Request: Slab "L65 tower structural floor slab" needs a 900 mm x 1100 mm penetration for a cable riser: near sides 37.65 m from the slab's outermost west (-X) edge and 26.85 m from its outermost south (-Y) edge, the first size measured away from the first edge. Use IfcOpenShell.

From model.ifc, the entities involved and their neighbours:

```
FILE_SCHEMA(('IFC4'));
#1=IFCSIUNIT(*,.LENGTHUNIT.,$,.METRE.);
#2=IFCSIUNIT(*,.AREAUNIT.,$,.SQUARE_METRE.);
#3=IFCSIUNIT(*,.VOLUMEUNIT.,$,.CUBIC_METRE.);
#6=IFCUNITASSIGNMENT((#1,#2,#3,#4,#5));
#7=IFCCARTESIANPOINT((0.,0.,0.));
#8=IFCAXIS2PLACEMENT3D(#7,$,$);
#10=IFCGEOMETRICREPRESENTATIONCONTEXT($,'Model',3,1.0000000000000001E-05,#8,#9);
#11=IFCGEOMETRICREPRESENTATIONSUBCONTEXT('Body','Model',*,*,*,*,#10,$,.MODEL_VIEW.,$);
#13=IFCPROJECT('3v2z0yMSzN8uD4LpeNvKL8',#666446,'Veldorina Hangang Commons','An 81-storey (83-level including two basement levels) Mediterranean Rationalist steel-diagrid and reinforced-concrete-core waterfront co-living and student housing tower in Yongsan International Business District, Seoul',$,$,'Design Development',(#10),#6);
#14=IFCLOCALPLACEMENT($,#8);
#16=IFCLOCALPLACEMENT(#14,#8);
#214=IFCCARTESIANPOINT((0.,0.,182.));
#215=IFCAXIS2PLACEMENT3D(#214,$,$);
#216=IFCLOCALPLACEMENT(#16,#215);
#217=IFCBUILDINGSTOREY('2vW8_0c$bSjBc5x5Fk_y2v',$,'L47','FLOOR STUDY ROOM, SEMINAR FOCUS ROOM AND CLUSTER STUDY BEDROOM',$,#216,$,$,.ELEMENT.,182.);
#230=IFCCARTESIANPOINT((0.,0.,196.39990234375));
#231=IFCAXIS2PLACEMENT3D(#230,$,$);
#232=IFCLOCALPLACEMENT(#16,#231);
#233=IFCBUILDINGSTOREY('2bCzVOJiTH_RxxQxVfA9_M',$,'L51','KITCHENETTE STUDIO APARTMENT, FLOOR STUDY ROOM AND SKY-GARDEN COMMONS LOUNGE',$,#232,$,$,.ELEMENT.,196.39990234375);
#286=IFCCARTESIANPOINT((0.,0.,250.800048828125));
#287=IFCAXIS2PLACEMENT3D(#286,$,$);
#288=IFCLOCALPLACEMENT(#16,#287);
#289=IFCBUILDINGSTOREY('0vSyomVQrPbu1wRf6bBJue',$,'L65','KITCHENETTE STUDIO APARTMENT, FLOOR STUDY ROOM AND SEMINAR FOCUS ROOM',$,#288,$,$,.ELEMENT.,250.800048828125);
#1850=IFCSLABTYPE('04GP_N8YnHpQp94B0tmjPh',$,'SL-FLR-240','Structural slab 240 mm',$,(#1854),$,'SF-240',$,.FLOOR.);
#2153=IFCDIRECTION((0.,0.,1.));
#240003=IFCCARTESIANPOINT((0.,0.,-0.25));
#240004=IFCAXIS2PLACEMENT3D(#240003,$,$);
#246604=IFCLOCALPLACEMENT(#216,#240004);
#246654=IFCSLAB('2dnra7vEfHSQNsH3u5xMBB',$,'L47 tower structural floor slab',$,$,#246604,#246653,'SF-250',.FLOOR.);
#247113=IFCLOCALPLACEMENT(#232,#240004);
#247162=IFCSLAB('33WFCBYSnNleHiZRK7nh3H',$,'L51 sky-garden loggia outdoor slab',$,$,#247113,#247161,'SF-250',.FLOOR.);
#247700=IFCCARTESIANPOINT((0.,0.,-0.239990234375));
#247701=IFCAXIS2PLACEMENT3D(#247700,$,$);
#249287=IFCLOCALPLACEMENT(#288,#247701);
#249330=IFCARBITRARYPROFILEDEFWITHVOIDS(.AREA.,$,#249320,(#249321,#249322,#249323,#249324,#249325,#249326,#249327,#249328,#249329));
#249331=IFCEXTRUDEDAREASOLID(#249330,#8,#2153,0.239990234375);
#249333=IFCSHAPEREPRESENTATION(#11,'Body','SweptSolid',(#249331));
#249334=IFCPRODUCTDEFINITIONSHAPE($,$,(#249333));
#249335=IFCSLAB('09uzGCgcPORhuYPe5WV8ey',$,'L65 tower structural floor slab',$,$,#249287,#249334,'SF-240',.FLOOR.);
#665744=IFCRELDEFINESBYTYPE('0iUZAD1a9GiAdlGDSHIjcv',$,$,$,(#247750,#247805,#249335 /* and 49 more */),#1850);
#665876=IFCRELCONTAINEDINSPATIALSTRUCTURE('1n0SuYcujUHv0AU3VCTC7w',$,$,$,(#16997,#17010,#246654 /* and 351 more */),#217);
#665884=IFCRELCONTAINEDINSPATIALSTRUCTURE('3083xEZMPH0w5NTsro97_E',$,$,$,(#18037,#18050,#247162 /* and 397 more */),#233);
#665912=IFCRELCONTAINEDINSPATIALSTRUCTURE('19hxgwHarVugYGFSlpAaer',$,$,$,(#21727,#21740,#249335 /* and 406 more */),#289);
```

```python
import numpy as np
import ifcopenshell
import ifcopenshell.api.feature
import ifcopenshell.api.geometry
import ifcopenshell.api.root
import ifcopenshell.geom
import ifcopenshell.util.placement
import ifcopenshell.util.representation
import ifcopenshell.util.shape
import ifcopenshell.util.unit

model = ifcopenshell.open("model.ifc")
unit_scale = ifcopenshell.util.unit.calculate_unit_scale(model)
settings = ifcopenshell.geom.settings()


def volume(element):
    """Net volume in cubic metres, openings subtracted."""
    shape = ifcopenshell.geom.create_shape(settings, element)
    return ifcopenshell.util.shape.get_volume(shape.geometry)


slab = model.by_id(249335)
before = volume(slab)

# Extent in the slab's own axes, in metres. The edges named are its -X and -Y sides.
slab_shape = ifcopenshell.geom.create_shape(settings, slab)
vertices = ifcopenshell.util.shape.get_vertices(slab_shape.geometry)
x_min, y_min, bottom = vertices.min(axis=0)
top = vertices[:, 2].max()

opening = ifcopenshell.api.root.create_entity(model, ifc_class="IfcOpeningElement", name="Cable riser opening", predefined_type="OPENING")
context = ifcopenshell.util.representation.get_context(model, "Model", "Body", "MODEL_VIEW")
width, depth = 0.9, 1.1
outline = [(0.0, 0.0), (width, 0.0), (width, depth), (0.0, depth), (0.0, 0.0)]
# Overshoot both faces by 50 mm so the cut is clean.
shape = ifcopenshell.api.geometry.add_slab_representation(
    model, context=context, depth=top - bottom + 0.1, polyline=outline
)
ifcopenshell.api.geometry.assign_representation(model, product=opening, representation=shape)

matrix = ifcopenshell.util.placement.get_local_placement(slab.ObjectPlacement)
matrix[:, 3] = matrix @ np.append(np.array([x_min + 37.65, y_min + 26.85, bottom - 0.05]) / unit_scale, 1.0)
ifcopenshell.api.geometry.edit_object_placement(model, product=opening, matrix=matrix, is_si=False)
ifcopenshell.api.feature.add_feature(model, feature=opening, element=slab)

after = volume(slab)

print(f"slab volume {before:.3f} -> {after:.3f} m3")

model.write("model_edited.ifc")
```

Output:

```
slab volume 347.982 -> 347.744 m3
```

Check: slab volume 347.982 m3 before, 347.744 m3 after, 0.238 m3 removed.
